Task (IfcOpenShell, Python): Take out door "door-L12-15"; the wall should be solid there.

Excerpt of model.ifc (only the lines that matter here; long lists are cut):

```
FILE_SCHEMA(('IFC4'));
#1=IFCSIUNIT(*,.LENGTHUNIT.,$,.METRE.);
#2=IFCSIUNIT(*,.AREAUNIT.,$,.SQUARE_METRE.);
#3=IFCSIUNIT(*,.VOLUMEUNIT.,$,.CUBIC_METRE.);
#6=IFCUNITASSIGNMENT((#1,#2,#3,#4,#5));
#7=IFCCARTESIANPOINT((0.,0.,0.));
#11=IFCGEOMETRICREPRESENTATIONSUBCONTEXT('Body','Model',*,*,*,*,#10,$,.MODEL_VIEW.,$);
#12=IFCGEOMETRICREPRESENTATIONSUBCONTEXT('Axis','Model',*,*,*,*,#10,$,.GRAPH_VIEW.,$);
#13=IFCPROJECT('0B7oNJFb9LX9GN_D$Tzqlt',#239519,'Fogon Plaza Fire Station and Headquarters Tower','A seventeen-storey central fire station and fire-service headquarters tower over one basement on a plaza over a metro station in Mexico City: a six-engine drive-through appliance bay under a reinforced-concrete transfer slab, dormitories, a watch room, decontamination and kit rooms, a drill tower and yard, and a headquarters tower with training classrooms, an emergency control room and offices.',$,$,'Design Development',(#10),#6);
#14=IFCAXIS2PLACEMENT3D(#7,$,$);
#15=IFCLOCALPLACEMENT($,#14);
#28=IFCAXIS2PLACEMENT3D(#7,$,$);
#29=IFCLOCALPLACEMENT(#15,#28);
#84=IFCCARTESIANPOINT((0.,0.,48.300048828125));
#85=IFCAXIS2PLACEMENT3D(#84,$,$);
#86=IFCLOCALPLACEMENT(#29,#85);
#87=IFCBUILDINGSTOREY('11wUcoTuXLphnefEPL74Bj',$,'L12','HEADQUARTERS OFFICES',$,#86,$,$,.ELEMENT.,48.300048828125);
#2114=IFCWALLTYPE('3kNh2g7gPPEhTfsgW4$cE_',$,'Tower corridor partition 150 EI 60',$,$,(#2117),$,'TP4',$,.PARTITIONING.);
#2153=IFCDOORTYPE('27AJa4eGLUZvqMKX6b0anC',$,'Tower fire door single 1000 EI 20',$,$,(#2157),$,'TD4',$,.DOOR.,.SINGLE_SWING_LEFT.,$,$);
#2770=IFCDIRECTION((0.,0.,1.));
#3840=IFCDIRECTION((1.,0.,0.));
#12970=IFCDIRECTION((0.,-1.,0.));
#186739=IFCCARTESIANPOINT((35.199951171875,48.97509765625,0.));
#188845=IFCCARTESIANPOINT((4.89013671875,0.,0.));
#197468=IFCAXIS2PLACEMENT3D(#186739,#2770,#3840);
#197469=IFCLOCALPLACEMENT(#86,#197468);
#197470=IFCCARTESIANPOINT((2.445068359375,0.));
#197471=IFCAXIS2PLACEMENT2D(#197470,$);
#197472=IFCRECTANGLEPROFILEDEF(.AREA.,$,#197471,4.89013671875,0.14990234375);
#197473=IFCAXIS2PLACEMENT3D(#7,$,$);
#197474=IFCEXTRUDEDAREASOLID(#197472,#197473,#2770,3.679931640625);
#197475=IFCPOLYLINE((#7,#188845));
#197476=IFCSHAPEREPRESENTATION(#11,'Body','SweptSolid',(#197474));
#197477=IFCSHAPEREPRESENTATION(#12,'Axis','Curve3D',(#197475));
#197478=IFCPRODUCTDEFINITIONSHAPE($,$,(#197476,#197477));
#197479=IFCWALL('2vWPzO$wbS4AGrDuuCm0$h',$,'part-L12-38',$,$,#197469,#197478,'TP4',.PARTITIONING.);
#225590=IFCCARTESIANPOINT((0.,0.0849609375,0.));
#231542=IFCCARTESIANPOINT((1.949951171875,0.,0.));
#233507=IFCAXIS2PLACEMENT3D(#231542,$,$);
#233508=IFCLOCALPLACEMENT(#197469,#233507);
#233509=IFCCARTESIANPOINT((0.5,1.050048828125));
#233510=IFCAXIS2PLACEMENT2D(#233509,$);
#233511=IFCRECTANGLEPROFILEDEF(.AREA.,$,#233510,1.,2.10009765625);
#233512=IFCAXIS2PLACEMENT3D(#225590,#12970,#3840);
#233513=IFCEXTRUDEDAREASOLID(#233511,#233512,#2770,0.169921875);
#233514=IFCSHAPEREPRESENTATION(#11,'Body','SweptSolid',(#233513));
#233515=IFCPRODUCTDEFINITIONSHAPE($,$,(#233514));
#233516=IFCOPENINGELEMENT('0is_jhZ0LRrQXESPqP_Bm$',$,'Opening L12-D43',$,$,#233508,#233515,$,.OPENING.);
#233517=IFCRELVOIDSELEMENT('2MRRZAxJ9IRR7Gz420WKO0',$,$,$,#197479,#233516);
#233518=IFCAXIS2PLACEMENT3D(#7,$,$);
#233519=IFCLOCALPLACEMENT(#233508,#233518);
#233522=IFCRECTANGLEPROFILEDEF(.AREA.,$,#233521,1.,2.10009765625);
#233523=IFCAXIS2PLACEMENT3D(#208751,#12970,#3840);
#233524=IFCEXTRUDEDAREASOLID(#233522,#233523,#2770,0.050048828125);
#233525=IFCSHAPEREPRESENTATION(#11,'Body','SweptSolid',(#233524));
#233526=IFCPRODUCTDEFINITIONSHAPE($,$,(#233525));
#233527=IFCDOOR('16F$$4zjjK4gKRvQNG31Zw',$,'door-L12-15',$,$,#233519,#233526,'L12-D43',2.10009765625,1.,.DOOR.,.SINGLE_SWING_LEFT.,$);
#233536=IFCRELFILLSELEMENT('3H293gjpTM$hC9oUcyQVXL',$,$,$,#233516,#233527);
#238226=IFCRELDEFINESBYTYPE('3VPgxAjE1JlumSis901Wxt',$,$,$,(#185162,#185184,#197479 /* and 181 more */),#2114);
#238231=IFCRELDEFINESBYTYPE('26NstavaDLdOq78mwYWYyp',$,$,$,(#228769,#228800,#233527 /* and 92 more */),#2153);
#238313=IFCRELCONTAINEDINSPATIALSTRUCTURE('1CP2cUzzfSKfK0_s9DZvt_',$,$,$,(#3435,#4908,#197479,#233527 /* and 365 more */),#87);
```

```python
import ifcopenshell
import ifcopenshell.api.feature
import ifcopenshell.api.root
import ifcopenshell.geom
import ifcopenshell.util.shape

model = ifcopenshell.open("model.ifc")
settings = ifcopenshell.geom.settings()


def volume(element):
    """Net volume in cubic metres, openings subtracted."""
    shape = ifcopenshell.geom.create_shape(settings, element)
    return ifcopenshell.util.shape.get_volume(shape.geometry)


door = model.by_guid("16F$$4zjjK4gKRvQNG31Zw")
opening = door.FillsVoids[0].RelatingOpeningElement
wall = opening.VoidsElements[0].RelatingBuildingElement
before = volume(wall)

ifcopenshell.api.root.remove_product(model, product=door)
ifcopenshell.api.feature.remove_feature(model, feature=opening)

after = volume(wall)

print(f"wall volume {before:.3f} -> {after:.3f} m3")

model.write("model_edited.ifc")
```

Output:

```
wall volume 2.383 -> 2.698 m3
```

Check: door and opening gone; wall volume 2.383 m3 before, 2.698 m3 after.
